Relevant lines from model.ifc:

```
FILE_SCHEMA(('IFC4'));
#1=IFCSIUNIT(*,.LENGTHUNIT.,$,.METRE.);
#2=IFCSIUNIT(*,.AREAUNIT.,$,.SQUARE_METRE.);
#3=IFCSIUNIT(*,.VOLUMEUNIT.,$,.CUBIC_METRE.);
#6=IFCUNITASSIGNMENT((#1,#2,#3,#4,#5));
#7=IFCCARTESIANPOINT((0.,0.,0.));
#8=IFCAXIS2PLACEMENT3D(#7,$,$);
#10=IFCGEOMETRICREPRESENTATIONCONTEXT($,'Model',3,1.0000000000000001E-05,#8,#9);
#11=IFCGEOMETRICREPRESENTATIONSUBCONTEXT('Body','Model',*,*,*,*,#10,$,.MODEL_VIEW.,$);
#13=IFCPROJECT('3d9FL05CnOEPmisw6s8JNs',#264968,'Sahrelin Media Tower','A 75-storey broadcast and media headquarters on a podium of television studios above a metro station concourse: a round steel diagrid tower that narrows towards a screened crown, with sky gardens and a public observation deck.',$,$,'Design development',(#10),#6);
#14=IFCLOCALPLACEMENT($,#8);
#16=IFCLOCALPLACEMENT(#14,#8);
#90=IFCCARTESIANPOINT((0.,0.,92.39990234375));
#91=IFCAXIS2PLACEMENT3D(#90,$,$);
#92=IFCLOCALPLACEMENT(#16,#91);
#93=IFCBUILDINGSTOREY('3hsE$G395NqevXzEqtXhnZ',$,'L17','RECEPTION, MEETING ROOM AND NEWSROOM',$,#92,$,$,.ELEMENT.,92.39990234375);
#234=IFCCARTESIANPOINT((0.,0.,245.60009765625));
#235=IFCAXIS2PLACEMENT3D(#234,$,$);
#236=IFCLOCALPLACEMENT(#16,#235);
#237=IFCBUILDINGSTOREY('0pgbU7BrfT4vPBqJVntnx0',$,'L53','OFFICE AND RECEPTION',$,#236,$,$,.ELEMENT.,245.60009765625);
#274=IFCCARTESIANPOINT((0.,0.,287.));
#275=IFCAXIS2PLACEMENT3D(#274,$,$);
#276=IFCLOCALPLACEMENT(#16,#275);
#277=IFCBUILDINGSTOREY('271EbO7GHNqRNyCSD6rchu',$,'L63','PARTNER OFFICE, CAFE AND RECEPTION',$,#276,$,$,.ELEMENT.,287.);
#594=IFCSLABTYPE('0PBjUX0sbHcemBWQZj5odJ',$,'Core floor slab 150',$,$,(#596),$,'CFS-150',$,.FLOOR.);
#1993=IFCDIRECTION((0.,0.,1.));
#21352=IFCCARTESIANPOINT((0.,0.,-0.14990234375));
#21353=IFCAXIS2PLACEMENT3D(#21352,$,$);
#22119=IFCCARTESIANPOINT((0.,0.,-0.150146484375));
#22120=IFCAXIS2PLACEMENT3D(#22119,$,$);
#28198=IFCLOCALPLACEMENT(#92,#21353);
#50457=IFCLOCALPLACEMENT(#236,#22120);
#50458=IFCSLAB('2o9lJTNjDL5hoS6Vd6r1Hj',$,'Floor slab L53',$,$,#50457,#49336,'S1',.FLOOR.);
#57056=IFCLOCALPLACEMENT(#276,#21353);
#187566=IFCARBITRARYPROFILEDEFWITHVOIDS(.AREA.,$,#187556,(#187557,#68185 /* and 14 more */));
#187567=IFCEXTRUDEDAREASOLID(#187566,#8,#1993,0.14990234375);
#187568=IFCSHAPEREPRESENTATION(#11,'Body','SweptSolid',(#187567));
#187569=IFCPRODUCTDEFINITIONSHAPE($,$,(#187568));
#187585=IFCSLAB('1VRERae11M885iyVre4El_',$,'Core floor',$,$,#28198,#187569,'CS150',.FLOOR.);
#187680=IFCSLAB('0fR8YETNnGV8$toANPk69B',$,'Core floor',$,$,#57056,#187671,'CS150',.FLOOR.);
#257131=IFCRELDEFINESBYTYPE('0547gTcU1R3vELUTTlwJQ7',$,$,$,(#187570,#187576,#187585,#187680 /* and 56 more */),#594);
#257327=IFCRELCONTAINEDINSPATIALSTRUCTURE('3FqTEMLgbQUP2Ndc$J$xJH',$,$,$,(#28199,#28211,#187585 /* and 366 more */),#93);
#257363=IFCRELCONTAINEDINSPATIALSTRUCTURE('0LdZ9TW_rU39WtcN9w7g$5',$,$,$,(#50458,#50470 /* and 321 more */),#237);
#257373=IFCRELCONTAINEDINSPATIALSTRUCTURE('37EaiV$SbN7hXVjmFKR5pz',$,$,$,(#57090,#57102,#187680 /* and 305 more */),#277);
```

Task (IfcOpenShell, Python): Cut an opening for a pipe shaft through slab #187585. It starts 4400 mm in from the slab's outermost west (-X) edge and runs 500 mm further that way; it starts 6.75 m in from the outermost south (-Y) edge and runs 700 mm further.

```python
import numpy as np
import ifcopenshell
import ifcopenshell.api.feature
import ifcopenshell.api.geometry
import ifcopenshell.api.root
import ifcopenshell.geom
import ifcopenshell.util.placement
import ifcopenshell.util.representation
import ifcopenshell.util.shape
import ifcopenshell.util.unit

model = ifcopenshell.open("model.ifc")
unit_scale = ifcopenshell.util.unit.calculate_unit_scale(model)
settings = ifcopenshell.geom.settings()


def volume(element):
    """Net volume in cubic metres, openings subtracted."""
    shape = ifcopenshell.geom.create_shape(settings, element)
    return ifcopenshell.util.shape.get_volume(shape.geometry)


slab = model.by_guid("1VRERae11M885iyVre4El_")
before = volume(slab)

# Extent in the slab's own axes, in metres. The edges named are its -X and -Y sides.
slab_shape = ifcopenshell.geom.create_shape(settings, slab)
vertices = ifcopenshell.util.shape.get_vertices(slab_shape.geometry)
x_min, y_min, bottom = vertices.min(axis=0)
top = vertices[:, 2].max()

opening = ifcopenshell.api.root.create_entity(model, ifc_class="IfcOpeningElement", name="Pipe shaft opening", predefined_type="OPENING")
context = ifcopenshell.util.representation.get_context(model, "Model", "Body", "MODEL_VIEW")
width, depth = 0.5, 0.7
outline = [(0.0, 0.0), (width, 0.0), (width, depth), (0.0, depth), (0.0, 0.0)]
# Overshoot both faces by 50 mm so the cut is clean.
shape = ifcopenshell.api.geometry.add_slab_representation(
    model, context=context, depth=top - bottom + 0.1, polyline=outline
)
ifcopenshell.api.geometry.assign_representation(model, product=opening, representation=shape)

matrix = ifcopenshell.util.placement.get_local_placement(slab.ObjectPlacement)
matrix[:, 3] = matrix @ np.append(np.array([x_min + 4.4, y_min + 6.75, bottom - 0.05]) / unit_scale, 1.0)
ifcopenshell.api.geometry.edit_object_placement(model, product=opening, matrix=matrix, is_si=False)
ifcopenshell.api.feature.add_feature(model, feature=opening, element=slab)

after = volume(slab)

print(f"slab volume {before:.3f} -> {after:.3f} m3")

model.write("model-out.ifc")
```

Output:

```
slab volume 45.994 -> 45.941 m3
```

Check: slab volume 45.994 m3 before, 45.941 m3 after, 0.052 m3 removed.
